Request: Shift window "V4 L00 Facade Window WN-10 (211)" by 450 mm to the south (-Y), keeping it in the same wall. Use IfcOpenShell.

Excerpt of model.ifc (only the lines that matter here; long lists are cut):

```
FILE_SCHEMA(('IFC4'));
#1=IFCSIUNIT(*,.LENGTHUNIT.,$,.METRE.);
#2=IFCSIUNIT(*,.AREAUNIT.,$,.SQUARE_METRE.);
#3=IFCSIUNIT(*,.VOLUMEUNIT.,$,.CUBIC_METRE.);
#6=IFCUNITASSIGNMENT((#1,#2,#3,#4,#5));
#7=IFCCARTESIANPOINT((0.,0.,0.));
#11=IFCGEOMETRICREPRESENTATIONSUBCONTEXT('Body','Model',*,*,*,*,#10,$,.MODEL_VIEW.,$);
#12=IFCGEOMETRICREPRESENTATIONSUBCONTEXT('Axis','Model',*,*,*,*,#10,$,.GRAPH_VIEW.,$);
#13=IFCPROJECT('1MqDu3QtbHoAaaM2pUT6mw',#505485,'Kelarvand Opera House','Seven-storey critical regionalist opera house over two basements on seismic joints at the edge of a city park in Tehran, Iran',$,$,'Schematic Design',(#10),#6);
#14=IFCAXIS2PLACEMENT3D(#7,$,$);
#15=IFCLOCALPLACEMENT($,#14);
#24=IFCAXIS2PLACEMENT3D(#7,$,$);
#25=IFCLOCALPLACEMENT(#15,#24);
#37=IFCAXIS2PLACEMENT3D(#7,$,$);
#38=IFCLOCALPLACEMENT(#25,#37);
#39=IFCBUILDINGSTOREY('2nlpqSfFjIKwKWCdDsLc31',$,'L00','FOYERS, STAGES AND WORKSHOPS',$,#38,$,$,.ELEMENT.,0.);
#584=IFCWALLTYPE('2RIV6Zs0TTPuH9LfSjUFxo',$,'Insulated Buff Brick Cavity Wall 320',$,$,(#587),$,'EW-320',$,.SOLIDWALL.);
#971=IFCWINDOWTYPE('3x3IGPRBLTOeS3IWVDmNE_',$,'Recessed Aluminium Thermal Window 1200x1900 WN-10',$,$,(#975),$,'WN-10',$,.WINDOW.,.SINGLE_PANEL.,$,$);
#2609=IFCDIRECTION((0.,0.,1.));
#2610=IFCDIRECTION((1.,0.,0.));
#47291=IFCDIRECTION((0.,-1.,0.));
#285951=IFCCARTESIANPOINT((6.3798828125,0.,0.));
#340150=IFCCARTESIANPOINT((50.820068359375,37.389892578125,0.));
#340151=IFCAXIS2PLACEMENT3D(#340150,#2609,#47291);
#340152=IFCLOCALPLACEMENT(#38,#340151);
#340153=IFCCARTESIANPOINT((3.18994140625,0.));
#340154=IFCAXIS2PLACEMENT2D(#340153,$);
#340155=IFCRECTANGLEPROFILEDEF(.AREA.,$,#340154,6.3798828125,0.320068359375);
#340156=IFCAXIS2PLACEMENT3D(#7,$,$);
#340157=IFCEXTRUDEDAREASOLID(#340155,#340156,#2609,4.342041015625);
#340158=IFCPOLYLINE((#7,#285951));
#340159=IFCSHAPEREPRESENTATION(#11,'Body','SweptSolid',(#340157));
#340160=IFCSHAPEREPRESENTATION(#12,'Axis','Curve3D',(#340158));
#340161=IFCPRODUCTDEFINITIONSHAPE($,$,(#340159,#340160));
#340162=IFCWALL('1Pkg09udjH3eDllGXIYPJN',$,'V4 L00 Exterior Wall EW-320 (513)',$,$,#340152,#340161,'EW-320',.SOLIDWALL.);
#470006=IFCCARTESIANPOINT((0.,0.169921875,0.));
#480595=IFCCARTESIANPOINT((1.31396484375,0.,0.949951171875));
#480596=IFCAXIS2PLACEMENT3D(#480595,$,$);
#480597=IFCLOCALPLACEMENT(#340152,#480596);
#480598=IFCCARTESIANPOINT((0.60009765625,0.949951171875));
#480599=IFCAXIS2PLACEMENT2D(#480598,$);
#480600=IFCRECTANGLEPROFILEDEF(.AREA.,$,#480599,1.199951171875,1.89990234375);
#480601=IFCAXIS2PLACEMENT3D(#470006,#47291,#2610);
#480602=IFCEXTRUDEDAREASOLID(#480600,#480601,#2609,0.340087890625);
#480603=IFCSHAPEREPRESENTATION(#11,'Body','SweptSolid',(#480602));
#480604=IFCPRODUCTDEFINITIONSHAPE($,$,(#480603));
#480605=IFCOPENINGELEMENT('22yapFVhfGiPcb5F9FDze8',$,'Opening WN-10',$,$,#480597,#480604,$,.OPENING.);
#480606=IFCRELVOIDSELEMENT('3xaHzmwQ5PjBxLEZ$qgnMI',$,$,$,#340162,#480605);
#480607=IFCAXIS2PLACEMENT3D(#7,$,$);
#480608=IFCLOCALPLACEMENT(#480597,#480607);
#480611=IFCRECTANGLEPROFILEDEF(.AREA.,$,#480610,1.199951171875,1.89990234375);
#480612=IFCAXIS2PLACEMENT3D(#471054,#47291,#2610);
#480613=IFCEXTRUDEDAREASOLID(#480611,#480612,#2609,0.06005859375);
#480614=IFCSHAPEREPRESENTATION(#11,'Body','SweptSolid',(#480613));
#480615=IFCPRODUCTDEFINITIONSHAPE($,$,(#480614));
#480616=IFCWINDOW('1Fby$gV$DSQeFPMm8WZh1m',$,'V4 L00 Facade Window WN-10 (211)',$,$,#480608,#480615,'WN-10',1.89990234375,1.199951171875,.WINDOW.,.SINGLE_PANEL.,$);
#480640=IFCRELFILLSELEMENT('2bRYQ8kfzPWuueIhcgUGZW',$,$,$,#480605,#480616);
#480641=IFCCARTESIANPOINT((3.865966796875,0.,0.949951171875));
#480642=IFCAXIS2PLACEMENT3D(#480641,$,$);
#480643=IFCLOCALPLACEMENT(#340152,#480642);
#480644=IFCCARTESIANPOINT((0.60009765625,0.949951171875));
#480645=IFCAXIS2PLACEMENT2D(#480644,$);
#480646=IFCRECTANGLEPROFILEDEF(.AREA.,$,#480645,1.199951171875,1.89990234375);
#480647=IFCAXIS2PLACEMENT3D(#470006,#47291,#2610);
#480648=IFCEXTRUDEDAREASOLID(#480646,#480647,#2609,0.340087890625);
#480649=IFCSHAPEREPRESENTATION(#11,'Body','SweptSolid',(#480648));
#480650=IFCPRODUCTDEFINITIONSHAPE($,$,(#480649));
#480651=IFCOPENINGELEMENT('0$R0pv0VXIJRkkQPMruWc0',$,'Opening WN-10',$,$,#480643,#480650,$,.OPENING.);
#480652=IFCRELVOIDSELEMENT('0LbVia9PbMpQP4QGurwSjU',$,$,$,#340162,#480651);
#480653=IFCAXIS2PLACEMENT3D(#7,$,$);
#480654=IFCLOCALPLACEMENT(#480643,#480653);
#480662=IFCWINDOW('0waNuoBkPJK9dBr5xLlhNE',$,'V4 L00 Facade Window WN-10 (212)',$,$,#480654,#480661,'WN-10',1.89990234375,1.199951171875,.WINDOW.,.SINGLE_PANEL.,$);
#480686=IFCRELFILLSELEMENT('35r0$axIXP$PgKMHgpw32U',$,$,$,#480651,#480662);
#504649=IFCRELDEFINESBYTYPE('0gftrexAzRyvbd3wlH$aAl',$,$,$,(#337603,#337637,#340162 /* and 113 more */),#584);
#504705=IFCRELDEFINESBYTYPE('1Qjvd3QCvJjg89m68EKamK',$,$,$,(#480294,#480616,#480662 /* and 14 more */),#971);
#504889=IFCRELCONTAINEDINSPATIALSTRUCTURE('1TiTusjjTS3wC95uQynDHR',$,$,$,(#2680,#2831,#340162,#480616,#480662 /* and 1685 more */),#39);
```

```python
import ifcopenshell
import ifcopenshell.api.geometry
import ifcopenshell.util.placement

model = ifcopenshell.open("model.ifc")

window = model.by_guid("1Fby$gV$DSQeFPMm8WZh1m")
opening = window.FillsVoids[0].RelatingOpeningElement
wall = opening.VoidsElements[0].RelatingBuildingElement

wall_matrix = ifcopenshell.util.placement.get_local_placement(wall.ObjectPlacement)
shift = wall_matrix[:3, 0] * 0.45
before = ifcopenshell.util.placement.get_local_placement(window.ObjectPlacement)[:3, 3].copy()

# The window is placed relative to its opening, so it follows when the opening moves.
matrix = ifcopenshell.util.placement.get_local_placement(opening.ObjectPlacement)
matrix[:3, 3] += shift
ifcopenshell.api.geometry.edit_object_placement(
    model, product=opening, matrix=matrix, is_si=False, should_transform_children=True
)

after = ifcopenshell.util.placement.get_local_placement(window.ObjectPlacement)[:3, 3]
print("window moved by", (after - before).round(3) + 0.0)

model.write("model_rev.ifc")
```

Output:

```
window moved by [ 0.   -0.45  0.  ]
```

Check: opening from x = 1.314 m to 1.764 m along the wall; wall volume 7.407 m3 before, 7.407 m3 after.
